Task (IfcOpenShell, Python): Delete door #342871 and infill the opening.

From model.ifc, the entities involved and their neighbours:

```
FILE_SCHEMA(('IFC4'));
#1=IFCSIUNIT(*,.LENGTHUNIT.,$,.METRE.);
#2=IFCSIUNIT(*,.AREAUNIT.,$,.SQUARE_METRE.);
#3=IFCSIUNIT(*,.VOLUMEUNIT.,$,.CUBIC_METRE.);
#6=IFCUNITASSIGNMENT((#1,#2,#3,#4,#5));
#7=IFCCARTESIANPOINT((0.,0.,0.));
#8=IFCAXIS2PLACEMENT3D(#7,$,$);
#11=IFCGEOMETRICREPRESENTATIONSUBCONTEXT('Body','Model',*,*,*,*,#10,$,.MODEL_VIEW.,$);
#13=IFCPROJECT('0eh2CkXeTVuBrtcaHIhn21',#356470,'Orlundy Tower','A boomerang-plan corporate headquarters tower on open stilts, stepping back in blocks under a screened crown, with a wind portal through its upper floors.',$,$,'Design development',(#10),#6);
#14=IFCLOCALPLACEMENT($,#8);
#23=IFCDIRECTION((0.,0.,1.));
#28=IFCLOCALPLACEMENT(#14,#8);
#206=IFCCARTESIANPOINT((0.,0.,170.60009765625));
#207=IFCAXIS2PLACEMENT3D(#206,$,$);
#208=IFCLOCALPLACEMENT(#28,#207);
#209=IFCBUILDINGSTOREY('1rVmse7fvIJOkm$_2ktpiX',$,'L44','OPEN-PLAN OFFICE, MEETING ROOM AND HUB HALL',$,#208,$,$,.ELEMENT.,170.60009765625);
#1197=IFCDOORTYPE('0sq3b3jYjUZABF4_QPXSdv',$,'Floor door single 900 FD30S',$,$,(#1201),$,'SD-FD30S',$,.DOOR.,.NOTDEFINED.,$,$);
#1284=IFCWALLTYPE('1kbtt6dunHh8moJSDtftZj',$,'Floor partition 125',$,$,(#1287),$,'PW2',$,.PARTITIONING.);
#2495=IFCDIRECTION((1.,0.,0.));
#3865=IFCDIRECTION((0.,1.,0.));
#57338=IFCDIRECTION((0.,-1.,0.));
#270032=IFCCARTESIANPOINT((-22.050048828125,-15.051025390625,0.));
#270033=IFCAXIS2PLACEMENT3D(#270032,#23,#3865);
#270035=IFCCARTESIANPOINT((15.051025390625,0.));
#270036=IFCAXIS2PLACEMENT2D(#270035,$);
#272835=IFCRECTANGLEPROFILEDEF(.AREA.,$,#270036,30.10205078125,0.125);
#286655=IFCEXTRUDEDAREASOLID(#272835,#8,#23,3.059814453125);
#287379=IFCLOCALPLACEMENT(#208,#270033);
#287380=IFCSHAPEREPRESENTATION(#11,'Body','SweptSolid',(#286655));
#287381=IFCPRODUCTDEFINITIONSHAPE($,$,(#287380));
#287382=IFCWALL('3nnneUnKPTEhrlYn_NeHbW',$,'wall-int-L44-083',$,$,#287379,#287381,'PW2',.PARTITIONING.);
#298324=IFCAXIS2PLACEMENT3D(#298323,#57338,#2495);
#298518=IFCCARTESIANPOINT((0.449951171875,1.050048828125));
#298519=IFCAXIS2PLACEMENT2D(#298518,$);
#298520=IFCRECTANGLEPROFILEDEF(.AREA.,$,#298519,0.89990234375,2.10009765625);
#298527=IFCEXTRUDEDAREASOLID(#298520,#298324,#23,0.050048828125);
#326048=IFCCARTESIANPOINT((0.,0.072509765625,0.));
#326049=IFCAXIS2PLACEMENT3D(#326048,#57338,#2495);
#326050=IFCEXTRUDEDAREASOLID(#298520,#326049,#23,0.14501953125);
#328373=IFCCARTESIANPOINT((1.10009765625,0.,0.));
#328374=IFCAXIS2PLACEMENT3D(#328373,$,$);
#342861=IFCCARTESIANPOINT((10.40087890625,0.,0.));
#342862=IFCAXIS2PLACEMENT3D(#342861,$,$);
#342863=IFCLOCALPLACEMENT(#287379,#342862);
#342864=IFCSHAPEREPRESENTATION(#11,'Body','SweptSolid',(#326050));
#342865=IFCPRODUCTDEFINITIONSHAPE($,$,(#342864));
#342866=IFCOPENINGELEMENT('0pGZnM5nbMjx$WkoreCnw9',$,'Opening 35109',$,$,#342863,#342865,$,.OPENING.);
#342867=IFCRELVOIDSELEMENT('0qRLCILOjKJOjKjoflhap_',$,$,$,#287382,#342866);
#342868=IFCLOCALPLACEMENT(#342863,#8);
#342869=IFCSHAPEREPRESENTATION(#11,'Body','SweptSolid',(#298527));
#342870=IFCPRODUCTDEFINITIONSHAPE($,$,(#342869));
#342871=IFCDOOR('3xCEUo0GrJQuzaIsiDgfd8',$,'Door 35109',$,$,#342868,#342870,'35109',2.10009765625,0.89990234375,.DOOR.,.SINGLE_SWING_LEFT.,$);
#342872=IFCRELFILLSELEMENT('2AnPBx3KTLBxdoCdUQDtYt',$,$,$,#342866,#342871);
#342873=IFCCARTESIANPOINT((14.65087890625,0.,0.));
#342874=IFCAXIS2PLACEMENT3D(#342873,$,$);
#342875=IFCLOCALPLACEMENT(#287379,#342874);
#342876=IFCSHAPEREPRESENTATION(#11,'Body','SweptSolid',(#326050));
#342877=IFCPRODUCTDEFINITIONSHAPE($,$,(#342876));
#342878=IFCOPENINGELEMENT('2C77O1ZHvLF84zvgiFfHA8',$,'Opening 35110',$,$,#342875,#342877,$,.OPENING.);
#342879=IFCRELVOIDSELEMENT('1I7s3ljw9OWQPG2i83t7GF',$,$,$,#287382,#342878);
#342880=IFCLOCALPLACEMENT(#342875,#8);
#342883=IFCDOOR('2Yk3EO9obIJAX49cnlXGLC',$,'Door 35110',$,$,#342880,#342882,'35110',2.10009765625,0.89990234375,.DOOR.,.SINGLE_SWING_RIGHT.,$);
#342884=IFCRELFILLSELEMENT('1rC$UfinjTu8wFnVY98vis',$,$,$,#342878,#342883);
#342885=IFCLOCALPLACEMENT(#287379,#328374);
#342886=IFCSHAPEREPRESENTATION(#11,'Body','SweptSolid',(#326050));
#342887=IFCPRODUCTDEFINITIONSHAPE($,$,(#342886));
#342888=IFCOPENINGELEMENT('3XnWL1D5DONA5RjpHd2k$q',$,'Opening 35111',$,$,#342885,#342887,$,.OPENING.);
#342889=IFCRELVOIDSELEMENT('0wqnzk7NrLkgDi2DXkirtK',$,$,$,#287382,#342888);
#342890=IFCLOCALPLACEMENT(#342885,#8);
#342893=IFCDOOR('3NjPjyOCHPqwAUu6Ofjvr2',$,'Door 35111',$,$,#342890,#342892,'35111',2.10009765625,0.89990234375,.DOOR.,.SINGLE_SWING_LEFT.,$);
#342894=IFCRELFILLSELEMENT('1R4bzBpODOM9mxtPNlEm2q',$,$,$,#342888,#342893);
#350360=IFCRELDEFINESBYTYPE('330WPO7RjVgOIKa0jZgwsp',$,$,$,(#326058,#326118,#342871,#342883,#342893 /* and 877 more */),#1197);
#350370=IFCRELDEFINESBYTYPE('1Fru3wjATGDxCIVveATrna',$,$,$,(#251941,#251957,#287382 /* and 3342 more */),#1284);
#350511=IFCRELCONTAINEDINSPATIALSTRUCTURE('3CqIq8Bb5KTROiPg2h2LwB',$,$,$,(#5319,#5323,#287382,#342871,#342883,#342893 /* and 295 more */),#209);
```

```python
import ifcopenshell
import ifcopenshell.api.feature
import ifcopenshell.api.root
import ifcopenshell.geom
import ifcopenshell.util.shape

model = ifcopenshell.open("model.ifc")
settings = ifcopenshell.geom.settings()


def volume(element):
    """Net volume in cubic metres, openings subtracted."""
    shape = ifcopenshell.geom.create_shape(settings, element)
    return ifcopenshell.util.shape.get_volume(shape.geometry)


door = model.by_guid("3xCEUo0GrJQuzaIsiDgfd8")
opening = door.FillsVoids[0].RelatingOpeningElement
wall = opening.VoidsElements[0].RelatingBuildingElement
before = volume(wall)

ifcopenshell.api.root.remove_product(model, product=door)
ifcopenshell.api.feature.remove_feature(model, feature=opening)

after = volume(wall)

print(f"wall volume {before:.3f} -> {after:.3f} m3")

model.write("model_updated.ifc")
```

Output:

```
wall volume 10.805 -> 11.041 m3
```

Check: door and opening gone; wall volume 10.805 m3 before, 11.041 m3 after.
